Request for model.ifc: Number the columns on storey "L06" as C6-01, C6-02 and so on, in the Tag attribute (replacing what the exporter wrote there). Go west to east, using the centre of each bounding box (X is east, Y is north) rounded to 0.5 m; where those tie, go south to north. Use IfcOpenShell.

First a look at what the model holds.

```python
import ifcopenshell
import ifcopenshell.util.element
import ifcopenshell.util.placement

model = ifcopenshell.open("model.ifc")
print(model.schema)
storey = next(s for s in model.by_type("IfcBuildingStorey") if s.Name == "L06")
columns = [e for e in ifcopenshell.util.element.get_decomposition(storey) if e.is_a("IfcColumn")]
for e in sorted(columns, key=lambda e: e.id()):
    origin = ifcopenshell.util.placement.get_local_placement(e.ObjectPlacement)[:3, 3]
    print(e.id(), e.Tag, e.Name, origin.round(2) + 0.0, sep=" | ")
```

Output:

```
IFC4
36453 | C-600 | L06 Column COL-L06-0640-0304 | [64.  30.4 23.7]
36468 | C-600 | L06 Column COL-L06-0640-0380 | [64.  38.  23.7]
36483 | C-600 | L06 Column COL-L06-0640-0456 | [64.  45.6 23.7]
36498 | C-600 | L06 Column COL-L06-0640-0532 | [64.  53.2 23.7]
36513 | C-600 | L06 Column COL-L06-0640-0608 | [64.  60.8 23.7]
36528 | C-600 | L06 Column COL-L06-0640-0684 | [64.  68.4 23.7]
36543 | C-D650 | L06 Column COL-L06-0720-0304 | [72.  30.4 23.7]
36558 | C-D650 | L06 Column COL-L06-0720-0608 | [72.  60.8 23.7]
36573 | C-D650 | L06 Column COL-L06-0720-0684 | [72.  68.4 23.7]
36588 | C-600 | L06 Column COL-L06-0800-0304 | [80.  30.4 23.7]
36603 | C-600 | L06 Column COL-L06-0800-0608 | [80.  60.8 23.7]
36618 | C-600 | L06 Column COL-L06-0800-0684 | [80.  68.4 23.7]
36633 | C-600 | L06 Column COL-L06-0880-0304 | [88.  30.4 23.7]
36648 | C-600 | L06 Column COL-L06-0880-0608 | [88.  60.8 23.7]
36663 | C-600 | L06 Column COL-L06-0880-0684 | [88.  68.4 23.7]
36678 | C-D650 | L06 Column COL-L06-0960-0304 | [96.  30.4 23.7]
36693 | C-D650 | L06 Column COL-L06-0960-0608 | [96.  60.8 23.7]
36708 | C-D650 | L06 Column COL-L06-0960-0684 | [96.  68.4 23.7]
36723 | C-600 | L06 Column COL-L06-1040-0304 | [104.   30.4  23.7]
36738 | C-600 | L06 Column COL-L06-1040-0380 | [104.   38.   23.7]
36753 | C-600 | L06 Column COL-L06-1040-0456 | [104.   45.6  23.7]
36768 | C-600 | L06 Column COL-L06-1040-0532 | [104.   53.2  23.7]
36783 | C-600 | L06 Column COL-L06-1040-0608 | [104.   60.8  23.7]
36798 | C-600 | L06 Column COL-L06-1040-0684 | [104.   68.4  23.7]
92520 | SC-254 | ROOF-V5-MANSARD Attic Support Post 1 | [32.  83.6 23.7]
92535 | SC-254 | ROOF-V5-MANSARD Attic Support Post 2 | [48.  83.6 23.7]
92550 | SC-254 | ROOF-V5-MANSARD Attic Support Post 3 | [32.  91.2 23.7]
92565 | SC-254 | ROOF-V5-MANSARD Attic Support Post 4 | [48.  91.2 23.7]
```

```python
import ifcopenshell
import ifcopenshell.geom
import ifcopenshell.util.element
import ifcopenshell.util.shape

model = ifcopenshell.open("model.ifc")
settings = ifcopenshell.geom.settings()
settings.set("use-world-coords", True)


def centre(element):
    shape = ifcopenshell.geom.create_shape(settings, element)
    return ifcopenshell.util.shape.get_bbox_centroid(shape.geometry)


storey = next(s for s in model.by_type("IfcBuildingStorey") if s.Name == "L06")
columns = [e for e in ifcopenshell.util.element.get_decomposition(storey) if e.is_a("IfcColumn")]

# Insertion points can sit at a corner or the storey origin, so sort by the geometry (in metres).
centres = {e: centre(e) for e in columns}
columns.sort(key=lambda e: (round(centres[e][0] / 0.5), centres[e][1]))

for i, e in enumerate(columns, start=1):
    number = f"C6-{i:02d}"
    e.Tag = number
    print(e.id(), number)

model.write("model-out.ifc")
```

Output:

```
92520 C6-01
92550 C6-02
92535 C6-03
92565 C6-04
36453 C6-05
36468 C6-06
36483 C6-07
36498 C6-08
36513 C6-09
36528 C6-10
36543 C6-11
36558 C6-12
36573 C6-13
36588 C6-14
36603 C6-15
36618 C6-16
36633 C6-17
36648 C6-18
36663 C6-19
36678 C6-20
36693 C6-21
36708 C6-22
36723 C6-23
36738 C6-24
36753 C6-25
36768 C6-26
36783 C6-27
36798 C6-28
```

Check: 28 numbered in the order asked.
